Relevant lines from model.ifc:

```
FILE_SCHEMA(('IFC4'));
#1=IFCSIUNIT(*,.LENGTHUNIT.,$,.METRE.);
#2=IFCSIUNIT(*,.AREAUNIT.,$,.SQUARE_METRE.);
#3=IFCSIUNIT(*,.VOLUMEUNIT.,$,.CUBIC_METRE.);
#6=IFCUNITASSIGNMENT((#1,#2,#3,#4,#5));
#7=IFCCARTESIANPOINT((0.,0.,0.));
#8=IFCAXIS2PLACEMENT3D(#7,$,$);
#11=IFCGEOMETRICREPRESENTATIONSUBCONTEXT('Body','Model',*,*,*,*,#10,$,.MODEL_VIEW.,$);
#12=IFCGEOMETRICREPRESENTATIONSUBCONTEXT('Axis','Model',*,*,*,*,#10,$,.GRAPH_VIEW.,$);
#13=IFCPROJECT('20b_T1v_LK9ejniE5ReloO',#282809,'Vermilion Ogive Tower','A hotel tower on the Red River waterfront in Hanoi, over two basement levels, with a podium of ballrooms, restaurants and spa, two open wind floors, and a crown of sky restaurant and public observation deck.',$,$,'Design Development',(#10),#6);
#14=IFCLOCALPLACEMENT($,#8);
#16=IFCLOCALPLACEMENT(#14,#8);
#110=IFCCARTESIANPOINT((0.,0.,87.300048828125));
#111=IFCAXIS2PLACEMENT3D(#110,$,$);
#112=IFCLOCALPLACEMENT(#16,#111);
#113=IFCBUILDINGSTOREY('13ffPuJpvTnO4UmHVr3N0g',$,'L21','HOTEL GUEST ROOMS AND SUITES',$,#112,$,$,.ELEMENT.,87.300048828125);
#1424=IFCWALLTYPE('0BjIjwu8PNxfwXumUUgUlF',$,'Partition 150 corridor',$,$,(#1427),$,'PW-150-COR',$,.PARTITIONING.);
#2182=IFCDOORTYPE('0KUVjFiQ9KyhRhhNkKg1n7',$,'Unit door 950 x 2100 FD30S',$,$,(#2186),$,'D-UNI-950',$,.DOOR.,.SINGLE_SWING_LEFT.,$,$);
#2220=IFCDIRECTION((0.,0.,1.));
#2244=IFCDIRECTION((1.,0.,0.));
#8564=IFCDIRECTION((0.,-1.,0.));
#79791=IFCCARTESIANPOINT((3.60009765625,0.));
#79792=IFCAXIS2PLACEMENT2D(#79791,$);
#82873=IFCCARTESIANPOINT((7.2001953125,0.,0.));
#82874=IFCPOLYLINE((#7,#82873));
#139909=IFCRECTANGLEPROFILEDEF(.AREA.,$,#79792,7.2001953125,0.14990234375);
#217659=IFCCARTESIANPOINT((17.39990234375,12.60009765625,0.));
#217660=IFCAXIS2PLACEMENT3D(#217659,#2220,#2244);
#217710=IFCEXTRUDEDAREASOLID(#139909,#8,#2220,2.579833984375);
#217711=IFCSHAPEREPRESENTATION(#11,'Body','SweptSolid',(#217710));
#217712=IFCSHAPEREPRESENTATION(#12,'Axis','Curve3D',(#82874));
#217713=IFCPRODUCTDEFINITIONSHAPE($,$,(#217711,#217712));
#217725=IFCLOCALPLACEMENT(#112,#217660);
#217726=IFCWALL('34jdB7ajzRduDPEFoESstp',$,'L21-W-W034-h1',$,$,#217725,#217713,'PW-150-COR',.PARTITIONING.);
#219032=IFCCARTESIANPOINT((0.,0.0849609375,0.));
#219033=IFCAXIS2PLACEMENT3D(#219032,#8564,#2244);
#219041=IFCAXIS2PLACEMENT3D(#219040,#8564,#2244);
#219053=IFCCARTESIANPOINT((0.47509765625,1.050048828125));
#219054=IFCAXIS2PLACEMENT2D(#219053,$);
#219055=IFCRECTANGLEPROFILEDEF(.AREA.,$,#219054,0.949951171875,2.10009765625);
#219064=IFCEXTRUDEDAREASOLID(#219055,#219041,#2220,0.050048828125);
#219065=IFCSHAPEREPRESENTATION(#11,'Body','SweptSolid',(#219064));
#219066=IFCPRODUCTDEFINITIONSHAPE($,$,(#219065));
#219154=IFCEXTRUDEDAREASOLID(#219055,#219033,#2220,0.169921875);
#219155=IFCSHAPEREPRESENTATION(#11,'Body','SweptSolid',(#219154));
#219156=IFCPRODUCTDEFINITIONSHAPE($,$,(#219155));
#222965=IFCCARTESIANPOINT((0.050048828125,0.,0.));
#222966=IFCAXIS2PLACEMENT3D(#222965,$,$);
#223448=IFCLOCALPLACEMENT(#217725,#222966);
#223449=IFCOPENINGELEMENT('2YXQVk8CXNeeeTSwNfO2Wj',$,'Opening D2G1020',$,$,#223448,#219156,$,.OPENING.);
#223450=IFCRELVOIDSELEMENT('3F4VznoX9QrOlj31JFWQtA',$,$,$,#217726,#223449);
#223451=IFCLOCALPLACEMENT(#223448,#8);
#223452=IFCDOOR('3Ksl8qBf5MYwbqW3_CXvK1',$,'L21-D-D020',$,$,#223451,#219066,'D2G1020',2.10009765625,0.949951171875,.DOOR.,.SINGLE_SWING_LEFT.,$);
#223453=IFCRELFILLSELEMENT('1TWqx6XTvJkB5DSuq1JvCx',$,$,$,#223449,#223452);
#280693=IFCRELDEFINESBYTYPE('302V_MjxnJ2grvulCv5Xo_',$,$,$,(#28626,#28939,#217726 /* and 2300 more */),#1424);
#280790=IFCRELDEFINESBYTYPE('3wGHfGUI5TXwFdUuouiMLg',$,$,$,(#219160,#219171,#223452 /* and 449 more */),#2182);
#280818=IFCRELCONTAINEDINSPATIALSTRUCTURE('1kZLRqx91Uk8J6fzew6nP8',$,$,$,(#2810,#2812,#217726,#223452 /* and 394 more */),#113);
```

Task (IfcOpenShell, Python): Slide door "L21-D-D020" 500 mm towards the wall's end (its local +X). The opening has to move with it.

```python
import ifcopenshell
import ifcopenshell.api.geometry
import ifcopenshell.util.placement

model = ifcopenshell.open("model.ifc")

door = model.by_guid("3Ksl8qBf5MYwbqW3_CXvK1")
opening = door.FillsVoids[0].RelatingOpeningElement
wall = opening.VoidsElements[0].RelatingBuildingElement

wall_matrix = ifcopenshell.util.placement.get_local_placement(wall.ObjectPlacement)
shift = wall_matrix[:3, 0] * 0.5
before = ifcopenshell.util.placement.get_local_placement(door.ObjectPlacement)[:3, 3].copy()

# The door is placed relative to its opening, so it follows when the opening moves.
matrix = ifcopenshell.util.placement.get_local_placement(opening.ObjectPlacement)
matrix[:3, 3] += shift
ifcopenshell.api.geometry.edit_object_placement(
    model, product=opening, matrix=matrix, is_si=False, should_transform_children=True
)

after = ifcopenshell.util.placement.get_local_placement(door.ObjectPlacement)[:3, 3]
print("door moved by", (after - before).round(3) + 0.0)

model.write("model_updated.ifc")
```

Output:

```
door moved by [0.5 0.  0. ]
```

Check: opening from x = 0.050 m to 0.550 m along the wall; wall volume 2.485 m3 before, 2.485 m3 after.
